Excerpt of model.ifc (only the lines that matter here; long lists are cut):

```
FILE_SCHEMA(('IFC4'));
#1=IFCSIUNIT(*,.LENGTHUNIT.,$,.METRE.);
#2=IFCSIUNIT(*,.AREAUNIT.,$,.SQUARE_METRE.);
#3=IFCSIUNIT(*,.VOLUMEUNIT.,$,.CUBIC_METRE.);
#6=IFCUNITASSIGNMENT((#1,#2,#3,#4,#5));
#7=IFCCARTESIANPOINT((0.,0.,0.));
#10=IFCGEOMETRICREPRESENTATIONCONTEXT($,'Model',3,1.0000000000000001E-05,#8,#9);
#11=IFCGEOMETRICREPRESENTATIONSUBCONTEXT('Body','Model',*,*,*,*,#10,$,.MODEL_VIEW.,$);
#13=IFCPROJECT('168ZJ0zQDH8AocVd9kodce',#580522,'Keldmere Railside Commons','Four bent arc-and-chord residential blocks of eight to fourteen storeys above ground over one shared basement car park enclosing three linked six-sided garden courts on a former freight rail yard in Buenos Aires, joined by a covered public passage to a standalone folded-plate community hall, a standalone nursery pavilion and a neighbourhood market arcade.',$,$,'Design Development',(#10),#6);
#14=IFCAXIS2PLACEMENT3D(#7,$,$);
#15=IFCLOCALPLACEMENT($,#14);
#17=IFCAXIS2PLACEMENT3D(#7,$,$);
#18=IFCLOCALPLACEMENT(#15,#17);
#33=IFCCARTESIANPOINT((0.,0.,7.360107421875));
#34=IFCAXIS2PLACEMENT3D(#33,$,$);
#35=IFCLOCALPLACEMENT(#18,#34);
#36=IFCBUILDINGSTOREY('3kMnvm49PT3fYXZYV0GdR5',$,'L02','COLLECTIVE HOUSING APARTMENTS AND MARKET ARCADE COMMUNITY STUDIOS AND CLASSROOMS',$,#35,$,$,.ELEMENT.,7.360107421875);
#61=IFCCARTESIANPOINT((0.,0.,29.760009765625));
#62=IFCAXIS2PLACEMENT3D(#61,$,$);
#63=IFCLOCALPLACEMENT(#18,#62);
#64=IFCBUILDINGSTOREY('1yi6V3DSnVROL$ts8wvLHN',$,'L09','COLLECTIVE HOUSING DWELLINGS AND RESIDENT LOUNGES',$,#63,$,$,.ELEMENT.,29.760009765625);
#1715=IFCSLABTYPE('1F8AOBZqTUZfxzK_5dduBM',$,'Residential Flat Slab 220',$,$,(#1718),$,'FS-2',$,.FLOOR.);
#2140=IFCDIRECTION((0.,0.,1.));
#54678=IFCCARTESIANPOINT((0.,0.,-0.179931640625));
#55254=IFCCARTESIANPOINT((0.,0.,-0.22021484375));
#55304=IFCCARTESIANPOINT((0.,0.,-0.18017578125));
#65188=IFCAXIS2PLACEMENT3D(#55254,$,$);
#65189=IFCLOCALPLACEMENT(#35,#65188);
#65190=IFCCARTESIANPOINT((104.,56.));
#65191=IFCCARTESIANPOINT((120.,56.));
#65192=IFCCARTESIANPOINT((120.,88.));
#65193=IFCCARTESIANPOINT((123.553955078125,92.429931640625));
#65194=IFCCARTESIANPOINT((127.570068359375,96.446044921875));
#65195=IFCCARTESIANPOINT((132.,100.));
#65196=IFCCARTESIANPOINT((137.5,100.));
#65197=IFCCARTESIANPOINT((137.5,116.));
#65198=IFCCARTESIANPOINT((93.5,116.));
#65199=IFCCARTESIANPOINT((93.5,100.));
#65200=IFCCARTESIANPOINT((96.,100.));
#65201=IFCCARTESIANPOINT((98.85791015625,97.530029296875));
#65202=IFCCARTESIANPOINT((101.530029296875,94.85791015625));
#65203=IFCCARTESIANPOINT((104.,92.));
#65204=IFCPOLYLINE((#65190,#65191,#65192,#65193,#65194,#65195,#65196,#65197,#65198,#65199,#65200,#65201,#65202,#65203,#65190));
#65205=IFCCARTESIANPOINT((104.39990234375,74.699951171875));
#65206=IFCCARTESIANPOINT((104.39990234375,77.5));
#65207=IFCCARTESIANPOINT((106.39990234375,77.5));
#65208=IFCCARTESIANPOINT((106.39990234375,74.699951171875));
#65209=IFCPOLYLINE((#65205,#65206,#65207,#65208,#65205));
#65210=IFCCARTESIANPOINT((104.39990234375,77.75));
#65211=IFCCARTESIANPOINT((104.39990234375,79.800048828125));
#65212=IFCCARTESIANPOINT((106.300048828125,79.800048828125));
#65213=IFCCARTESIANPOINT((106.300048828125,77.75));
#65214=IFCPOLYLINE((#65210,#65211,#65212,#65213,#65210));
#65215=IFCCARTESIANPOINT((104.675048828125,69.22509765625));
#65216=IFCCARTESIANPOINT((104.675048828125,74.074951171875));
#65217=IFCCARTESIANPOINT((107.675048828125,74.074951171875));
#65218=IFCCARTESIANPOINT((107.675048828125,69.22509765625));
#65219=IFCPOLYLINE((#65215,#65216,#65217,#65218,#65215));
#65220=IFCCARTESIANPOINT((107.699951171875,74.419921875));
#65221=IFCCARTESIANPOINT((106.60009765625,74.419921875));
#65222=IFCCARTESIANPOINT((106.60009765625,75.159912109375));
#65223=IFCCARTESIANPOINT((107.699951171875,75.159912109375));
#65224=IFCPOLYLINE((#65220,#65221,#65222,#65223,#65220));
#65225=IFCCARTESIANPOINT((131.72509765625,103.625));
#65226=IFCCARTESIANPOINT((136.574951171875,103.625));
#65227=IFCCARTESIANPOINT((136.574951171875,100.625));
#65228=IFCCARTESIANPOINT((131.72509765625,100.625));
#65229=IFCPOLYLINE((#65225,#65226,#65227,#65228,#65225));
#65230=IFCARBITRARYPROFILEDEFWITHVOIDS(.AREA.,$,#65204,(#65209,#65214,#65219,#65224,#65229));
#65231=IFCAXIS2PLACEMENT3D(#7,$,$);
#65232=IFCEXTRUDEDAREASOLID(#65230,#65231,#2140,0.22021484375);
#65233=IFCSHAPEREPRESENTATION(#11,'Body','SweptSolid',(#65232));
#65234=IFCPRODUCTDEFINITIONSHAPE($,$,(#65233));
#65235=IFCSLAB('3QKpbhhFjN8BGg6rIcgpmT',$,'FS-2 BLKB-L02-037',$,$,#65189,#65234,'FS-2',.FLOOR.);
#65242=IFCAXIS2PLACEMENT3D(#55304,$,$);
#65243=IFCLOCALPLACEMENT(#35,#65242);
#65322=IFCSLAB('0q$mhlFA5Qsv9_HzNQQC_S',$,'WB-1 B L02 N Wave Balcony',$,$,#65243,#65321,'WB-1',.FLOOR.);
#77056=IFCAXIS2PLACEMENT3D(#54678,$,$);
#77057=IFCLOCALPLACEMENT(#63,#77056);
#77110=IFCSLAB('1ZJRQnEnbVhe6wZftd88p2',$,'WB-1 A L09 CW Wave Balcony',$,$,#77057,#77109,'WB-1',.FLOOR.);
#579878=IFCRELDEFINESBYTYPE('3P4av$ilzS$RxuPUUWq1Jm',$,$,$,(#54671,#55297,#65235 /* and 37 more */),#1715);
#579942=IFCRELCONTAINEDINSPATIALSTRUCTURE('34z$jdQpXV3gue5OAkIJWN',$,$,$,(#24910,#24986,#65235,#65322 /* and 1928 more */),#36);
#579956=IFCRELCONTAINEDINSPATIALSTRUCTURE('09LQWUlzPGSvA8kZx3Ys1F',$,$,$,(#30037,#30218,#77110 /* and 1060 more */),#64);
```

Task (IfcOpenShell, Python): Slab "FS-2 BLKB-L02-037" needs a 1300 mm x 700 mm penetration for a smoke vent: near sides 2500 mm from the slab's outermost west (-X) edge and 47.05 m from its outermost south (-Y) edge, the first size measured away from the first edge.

```python
import numpy as np
import ifcopenshell
import ifcopenshell.api.feature
import ifcopenshell.api.geometry
import ifcopenshell.api.root
import ifcopenshell.geom
import ifcopenshell.util.placement
import ifcopenshell.util.representation
import ifcopenshell.util.shape
import ifcopenshell.util.unit

model = ifcopenshell.open("model.ifc")
unit_scale = ifcopenshell.util.unit.calculate_unit_scale(model)
settings = ifcopenshell.geom.settings()


def volume(element):
    """Net volume in cubic metres, openings subtracted."""
    shape = ifcopenshell.geom.create_shape(settings, element)
    return ifcopenshell.util.shape.get_volume(shape.geometry)


slab = model.by_guid("3QKpbhhFjN8BGg6rIcgpmT")
before = volume(slab)

# Extent in the slab's own axes, in metres. The edges named are its -X and -Y sides.
slab_shape = ifcopenshell.geom.create_shape(settings, slab)
vertices = ifcopenshell.util.shape.get_vertices(slab_shape.geometry)
x_min, y_min, bottom = vertices.min(axis=0)
top = vertices[:, 2].max()

opening = ifcopenshell.api.root.create_entity(model, ifc_class="IfcOpeningElement", name="Smoke vent opening", predefined_type="OPENING")
context = ifcopenshell.util.representation.get_context(model, "Model", "Body", "MODEL_VIEW")
width, depth = 1.3, 0.7
outline = [(0.0, 0.0), (width, 0.0), (width, depth), (0.0, depth), (0.0, 0.0)]
# Overshoot both faces by 50 mm so the cut is clean.
shape = ifcopenshell.api.geometry.add_slab_representation(
    model, context=context, depth=top - bottom + 0.1, polyline=outline
)
ifcopenshell.api.geometry.assign_representation(model, product=opening, representation=shape)

matrix = ifcopenshell.util.placement.get_local_placement(slab.ObjectPlacement)
matrix[:, 3] = matrix @ np.append(np.array([x_min + 2.5, y_min + 47.05, bottom - 0.05]) / unit_scale, 1.0)
ifcopenshell.api.geometry.edit_object_placement(model, product=opening, matrix=matrix, is_si=False)
ifcopenshell.api.feature.add_feature(model, feature=opening, element=slab)

after = volume(slab)

print(f"slab volume {before:.3f} -> {after:.3f} m3")

model.write("model-out.ifc")
```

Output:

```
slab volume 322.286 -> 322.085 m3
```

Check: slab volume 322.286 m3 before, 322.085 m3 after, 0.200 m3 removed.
